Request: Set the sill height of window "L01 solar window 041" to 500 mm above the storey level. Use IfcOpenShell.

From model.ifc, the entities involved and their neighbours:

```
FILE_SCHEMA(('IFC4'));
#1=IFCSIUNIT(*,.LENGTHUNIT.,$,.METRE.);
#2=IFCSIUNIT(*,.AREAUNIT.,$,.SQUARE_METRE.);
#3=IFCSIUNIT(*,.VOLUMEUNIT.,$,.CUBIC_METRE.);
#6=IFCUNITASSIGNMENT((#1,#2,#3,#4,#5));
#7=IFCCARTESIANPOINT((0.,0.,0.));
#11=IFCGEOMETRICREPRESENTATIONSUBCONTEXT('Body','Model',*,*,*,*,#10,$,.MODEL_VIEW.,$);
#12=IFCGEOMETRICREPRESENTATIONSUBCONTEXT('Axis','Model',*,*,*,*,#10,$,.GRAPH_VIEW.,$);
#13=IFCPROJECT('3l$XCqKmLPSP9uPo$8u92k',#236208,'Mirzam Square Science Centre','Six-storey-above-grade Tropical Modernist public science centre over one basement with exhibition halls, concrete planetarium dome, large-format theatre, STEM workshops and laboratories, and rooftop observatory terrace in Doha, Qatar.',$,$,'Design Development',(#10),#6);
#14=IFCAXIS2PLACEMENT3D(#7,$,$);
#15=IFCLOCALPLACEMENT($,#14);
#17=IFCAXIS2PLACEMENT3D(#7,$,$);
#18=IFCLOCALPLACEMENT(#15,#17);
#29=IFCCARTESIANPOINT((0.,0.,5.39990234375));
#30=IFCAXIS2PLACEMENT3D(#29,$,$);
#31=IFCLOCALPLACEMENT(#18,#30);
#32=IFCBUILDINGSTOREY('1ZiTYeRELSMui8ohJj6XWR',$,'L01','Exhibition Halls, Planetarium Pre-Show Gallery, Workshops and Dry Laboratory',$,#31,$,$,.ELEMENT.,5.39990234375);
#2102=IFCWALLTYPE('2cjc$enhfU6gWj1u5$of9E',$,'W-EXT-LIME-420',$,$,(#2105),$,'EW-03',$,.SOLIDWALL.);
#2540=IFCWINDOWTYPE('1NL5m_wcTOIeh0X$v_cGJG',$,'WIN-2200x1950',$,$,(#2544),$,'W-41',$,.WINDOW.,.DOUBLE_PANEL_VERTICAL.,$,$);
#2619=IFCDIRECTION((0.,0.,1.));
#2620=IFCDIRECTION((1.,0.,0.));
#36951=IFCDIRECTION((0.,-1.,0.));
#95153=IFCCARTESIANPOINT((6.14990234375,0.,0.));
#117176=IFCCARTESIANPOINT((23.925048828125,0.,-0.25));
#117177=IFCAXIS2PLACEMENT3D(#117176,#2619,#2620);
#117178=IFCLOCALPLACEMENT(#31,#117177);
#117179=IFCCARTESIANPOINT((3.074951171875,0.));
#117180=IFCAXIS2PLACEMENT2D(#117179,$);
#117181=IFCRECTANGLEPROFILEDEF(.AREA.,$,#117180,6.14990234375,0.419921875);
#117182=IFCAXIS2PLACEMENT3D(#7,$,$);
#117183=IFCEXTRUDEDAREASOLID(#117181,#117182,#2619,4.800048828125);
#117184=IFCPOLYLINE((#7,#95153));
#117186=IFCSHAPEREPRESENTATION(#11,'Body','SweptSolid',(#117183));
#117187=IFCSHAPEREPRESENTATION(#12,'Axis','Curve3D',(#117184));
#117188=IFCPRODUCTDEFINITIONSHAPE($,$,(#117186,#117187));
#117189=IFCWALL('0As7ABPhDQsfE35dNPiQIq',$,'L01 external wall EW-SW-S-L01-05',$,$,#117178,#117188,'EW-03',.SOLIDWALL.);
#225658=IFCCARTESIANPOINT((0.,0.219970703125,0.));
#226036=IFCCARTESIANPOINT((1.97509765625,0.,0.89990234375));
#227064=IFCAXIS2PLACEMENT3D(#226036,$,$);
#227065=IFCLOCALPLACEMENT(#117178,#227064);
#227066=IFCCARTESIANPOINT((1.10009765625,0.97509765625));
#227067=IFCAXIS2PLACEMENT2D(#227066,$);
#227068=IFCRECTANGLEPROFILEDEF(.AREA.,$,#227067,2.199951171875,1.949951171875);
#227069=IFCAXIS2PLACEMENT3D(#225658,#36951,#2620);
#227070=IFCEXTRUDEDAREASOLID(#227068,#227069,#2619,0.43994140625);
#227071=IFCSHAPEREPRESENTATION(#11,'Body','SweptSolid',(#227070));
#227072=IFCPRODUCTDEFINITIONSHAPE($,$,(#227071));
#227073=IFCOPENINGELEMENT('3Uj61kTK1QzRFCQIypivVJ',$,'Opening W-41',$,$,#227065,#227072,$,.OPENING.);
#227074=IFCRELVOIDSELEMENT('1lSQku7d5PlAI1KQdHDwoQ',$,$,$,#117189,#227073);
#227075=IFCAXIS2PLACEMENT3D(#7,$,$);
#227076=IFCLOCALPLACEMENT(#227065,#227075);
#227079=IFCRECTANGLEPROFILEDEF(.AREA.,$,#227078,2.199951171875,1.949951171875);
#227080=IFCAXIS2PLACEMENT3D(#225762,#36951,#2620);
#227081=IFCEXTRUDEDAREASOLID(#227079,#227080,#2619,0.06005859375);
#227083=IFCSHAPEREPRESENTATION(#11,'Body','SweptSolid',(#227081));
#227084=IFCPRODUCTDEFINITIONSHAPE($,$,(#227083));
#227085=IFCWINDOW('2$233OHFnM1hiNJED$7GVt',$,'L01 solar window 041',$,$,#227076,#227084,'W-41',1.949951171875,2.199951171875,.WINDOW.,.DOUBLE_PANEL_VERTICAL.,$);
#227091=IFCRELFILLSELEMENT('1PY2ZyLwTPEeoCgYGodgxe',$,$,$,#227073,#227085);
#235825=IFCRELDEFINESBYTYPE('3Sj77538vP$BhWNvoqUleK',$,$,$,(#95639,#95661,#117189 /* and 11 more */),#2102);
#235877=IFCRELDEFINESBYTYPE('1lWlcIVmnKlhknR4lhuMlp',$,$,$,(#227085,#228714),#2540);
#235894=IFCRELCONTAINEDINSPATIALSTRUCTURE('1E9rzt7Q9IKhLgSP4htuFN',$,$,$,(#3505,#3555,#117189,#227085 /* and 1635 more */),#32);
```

```python
import numpy as np
import ifcopenshell
import ifcopenshell.api.geometry
import ifcopenshell.geom
import ifcopenshell.util.element
import ifcopenshell.util.placement
import ifcopenshell.util.shape
import ifcopenshell.util.unit

model = ifcopenshell.open("model.ifc")
unit_scale = ifcopenshell.util.unit.calculate_unit_scale(model)

window = model.by_id(227085)
opening = window.FillsVoids[0].RelatingOpeningElement
storey = ifcopenshell.util.element.get_container(window, ifc_class="IfcBuildingStorey")
level = ifcopenshell.util.placement.get_local_placement(storey.ObjectPlacement)[2, 3]

# The opening's origin need not be at the sill, so measure its lowest point.
shape = ifcopenshell.geom.create_shape(ifcopenshell.geom.settings(), opening)
bottom = ifcopenshell.util.shape.get_shape_bottom_elevation(shape, shape.geometry) / unit_scale
dz = level + 0.5 - bottom

shift = np.array([0.0, 0.0, dz])
# The window is placed relative to its opening, so it follows when the opening moves.
matrix = ifcopenshell.util.placement.get_local_placement(opening.ObjectPlacement)
matrix[:3, 3] += shift
ifcopenshell.api.geometry.edit_object_placement(
    model, product=opening, matrix=matrix, is_si=False, should_transform_children=True
)

print(f"moved by {dz * unit_scale:+.3f} m")

model.write("model_edited.ifc")
```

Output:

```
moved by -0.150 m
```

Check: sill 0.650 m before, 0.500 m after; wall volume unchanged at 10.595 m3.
